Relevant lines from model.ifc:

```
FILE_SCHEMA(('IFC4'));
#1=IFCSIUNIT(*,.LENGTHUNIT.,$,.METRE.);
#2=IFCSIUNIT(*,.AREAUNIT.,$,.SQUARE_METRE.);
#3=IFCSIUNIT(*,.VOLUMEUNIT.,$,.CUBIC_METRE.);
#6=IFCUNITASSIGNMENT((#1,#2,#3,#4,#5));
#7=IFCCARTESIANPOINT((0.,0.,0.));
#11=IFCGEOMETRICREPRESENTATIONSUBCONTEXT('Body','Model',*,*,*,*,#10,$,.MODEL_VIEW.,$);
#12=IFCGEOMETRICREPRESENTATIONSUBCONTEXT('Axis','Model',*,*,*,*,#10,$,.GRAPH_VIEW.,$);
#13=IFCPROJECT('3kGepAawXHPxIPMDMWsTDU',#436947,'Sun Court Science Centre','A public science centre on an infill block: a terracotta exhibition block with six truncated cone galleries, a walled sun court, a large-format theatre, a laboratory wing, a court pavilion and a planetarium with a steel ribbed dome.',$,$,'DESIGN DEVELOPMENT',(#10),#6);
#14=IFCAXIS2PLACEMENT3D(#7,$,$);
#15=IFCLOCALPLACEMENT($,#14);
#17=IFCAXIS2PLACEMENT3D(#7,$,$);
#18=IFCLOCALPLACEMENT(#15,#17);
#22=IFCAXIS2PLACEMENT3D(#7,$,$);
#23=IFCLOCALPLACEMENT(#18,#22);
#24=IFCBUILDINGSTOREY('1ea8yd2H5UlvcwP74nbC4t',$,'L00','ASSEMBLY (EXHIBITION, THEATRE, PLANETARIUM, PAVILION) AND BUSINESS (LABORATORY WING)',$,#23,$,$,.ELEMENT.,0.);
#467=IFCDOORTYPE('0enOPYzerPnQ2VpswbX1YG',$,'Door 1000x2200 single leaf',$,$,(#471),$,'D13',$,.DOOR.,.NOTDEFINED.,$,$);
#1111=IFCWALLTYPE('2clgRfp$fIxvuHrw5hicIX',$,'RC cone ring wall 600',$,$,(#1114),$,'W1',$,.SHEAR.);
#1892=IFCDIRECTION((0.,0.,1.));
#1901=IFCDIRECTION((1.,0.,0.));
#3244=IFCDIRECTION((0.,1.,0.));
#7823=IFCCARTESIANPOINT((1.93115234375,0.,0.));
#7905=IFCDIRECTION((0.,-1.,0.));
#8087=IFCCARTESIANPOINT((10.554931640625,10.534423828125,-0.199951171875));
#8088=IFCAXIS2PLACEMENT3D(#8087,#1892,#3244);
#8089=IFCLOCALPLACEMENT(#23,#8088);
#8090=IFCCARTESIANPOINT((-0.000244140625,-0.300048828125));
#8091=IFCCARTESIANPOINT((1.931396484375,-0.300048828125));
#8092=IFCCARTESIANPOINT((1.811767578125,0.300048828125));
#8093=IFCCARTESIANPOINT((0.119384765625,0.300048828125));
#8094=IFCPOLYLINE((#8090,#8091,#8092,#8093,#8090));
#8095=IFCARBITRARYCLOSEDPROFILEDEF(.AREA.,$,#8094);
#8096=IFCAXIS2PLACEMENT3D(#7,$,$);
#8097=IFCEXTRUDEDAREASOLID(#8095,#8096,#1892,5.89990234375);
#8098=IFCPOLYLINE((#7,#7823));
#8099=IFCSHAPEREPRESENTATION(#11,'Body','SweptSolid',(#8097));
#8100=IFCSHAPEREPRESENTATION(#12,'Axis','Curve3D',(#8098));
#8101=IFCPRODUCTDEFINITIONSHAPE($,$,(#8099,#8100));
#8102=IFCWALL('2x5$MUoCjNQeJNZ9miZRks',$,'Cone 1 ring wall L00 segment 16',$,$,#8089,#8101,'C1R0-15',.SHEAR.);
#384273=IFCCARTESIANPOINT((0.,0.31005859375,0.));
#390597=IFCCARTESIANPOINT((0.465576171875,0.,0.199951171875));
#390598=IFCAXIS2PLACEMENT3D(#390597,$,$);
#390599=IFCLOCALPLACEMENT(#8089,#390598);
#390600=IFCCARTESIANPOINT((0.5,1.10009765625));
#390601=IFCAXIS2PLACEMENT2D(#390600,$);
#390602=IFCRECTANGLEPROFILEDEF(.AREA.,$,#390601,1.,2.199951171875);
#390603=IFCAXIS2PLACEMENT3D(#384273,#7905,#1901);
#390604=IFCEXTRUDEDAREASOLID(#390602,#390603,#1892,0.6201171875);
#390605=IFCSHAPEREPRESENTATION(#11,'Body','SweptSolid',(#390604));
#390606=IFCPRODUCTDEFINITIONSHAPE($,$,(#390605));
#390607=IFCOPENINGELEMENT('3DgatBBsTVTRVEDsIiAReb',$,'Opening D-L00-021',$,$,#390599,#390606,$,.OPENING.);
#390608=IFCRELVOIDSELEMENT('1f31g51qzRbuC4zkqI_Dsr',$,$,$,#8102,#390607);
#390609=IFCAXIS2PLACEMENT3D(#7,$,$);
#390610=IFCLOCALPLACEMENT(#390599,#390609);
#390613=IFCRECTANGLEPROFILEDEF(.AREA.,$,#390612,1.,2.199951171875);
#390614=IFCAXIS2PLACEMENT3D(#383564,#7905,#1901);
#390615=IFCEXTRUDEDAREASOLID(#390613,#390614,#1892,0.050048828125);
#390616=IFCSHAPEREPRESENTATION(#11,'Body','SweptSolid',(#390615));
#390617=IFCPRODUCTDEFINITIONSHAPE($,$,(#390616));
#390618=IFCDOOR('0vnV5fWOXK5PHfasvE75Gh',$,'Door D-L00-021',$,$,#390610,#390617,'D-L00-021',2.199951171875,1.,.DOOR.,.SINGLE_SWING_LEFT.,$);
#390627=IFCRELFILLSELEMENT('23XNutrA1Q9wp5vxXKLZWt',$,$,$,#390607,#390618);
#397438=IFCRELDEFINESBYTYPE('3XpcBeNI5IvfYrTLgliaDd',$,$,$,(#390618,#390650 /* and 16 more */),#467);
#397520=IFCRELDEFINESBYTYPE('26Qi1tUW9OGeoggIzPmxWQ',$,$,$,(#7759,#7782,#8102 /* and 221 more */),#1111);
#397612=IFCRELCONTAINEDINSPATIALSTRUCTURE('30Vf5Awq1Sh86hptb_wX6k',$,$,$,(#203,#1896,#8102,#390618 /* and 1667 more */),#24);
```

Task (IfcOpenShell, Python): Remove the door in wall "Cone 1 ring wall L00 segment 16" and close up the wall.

```python
import ifcopenshell
import ifcopenshell.api.feature
import ifcopenshell.api.root
import ifcopenshell.geom
import ifcopenshell.util.shape

model = ifcopenshell.open("model.ifc")
settings = ifcopenshell.geom.settings()


def volume(element):
    """Net volume in cubic metres, openings subtracted."""
    shape = ifcopenshell.geom.create_shape(settings, element)
    return ifcopenshell.util.shape.get_volume(shape.geometry)


door = model.by_guid("0vnV5fWOXK5PHfasvE75Gh")
opening = door.FillsVoids[0].RelatingOpeningElement
wall = opening.VoidsElements[0].RelatingBuildingElement
before = volume(wall)

ifcopenshell.api.root.remove_product(model, product=door)
ifcopenshell.api.feature.remove_feature(model, feature=opening)

after = volume(wall)

print(f"wall volume {before:.3f} -> {after:.3f} m3")

model.write("model_v2.ifc")
```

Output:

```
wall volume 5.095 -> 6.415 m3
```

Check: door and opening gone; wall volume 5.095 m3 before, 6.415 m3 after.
